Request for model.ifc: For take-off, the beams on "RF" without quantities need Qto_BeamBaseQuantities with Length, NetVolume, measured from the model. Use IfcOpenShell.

First a look at what the model holds.

```python
import ifcopenshell
import ifcopenshell.util.element
import ifcopenshell.util.unit

model = ifcopenshell.open("model.ifc")
print(model.schema)
for unit_type in ("LENGTHUNIT", "AREAUNIT", "VOLUMEUNIT"):
    print(unit_type, ifcopenshell.util.unit.calculate_unit_scale(model, unit_type))
storey = next(s for s in model.by_type("IfcBuildingStorey") if s.Name == "RF")
beams = [e for e in ifcopenshell.util.element.get_decomposition(storey) if e.is_a("IfcBeam")]
for e in sorted(beams, key=lambda e: e.id()):
    print(e.id(), e.is_a(), e.Name, list(ifcopenshell.util.element.get_psets(e, qtos_only=True)), sep=" | ")
```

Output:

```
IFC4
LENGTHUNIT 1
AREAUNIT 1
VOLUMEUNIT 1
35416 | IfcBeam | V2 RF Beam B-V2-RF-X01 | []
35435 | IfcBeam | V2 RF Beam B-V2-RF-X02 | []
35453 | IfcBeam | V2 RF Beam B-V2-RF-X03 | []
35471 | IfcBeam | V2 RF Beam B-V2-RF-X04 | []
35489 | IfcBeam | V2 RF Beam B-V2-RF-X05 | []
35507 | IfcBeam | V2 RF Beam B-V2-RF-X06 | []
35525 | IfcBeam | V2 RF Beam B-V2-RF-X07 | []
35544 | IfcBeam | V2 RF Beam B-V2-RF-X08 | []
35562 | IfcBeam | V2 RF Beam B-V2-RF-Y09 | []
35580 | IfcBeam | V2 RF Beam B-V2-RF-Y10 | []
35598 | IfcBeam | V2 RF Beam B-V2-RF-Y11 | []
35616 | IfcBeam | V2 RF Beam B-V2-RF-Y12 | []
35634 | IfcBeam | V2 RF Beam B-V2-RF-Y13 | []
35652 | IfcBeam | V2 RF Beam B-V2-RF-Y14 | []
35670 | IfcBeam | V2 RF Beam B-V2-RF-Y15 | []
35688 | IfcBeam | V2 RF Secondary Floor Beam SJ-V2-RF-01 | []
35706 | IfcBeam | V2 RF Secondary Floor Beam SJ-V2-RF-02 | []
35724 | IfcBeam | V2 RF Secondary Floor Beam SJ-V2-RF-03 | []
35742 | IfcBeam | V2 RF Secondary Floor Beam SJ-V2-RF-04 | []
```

```python
import ifcopenshell
import ifcopenshell.api.pset
import ifcopenshell.geom
import ifcopenshell.util.element
import ifcopenshell.util.shape
import ifcopenshell.util.unit

model = ifcopenshell.open("model.ifc")
unit_scale = ifcopenshell.util.unit.calculate_unit_scale(model)
volume_scale = ifcopenshell.util.unit.calculate_unit_scale(model, "VOLUMEUNIT")
settings = ifcopenshell.geom.settings()

storey = next(s for s in model.by_type("IfcBuildingStorey") if s.Name == "RF")
beams = [e for e in ifcopenshell.util.element.get_decomposition(storey) if e.is_a("IfcBeam")]

for e in sorted(beams, key=lambda e: e.id()):
    if ifcopenshell.util.element.get_psets(e, qtos_only=True, should_inherit=False):
        continue
    # Geometry comes back in metres, in the element's own axes.
    shape = ifcopenshell.geom.create_shape(settings, e)
    values = {
        "Length": ifcopenshell.util.shape.get_max_xyz(shape.geometry) / unit_scale,
        "NetVolume": ifcopenshell.util.shape.get_volume(shape.geometry) / volume_scale,
    }
    qto = ifcopenshell.api.pset.add_qto(model, product=e, name="Qto_BeamBaseQuantities")
    ifcopenshell.api.pset.edit_qto(model, qto=qto, properties=values)
    print(e.id(), {k: round(v, 3) for k, v in values.items()})

model.write("model-out.ifc")
```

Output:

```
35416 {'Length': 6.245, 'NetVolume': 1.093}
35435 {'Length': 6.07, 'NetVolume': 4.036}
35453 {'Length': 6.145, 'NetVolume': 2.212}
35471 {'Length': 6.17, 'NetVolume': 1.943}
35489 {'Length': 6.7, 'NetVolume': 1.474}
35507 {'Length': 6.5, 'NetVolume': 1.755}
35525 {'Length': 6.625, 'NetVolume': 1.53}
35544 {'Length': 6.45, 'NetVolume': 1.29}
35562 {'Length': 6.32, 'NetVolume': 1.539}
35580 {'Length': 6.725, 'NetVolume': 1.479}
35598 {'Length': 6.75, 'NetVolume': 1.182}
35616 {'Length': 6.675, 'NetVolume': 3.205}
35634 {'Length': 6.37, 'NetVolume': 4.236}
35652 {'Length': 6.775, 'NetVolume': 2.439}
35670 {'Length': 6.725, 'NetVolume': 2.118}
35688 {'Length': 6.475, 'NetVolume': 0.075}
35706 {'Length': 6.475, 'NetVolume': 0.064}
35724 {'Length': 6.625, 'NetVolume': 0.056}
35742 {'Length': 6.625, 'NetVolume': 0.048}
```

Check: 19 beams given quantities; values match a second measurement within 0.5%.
